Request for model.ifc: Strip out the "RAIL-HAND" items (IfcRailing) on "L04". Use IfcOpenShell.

First a look at what the model holds.

```python
import ifcopenshell
import ifcopenshell.util.element

model = ifcopenshell.open("model.ifc")
print(model.schema)
storey = next(s for s in model.by_type("IfcBuildingStorey") if s.Name == "L04")
railings = [e for e in ifcopenshell.util.element.get_decomposition(storey) if e.is_a("IfcRailing")]
seen = {}
for e in railings:
    element_type = ifcopenshell.util.element.get_type(e)
    name = element_type.Name if element_type not in (None, e) else None
    seen[name] = seen.get(name, 0) + 1
for name, count in sorted(seen.items(), key=str):
    print(count, "x", name)
```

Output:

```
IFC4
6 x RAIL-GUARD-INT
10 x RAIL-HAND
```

```python
import ifcopenshell
import ifcopenshell.api.root
import ifcopenshell.util.element

model = ifcopenshell.open("model.ifc")

storey = next(s for s in model.by_type("IfcBuildingStorey") if s.Name == "L04")
railings = [e for e in ifcopenshell.util.element.get_decomposition(storey) if e.is_a("IfcRailing")]
targets = [e for e in railings if (t := ifcopenshell.util.element.get_type(e)) not in (None, e) and t.Name == "RAIL-HAND"]

for e in targets:
    ifcopenshell.api.root.remove_product(model, product=e)
print(len(targets), "removed")

model.write("model_edited.ifc")
```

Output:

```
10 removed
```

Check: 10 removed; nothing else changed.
